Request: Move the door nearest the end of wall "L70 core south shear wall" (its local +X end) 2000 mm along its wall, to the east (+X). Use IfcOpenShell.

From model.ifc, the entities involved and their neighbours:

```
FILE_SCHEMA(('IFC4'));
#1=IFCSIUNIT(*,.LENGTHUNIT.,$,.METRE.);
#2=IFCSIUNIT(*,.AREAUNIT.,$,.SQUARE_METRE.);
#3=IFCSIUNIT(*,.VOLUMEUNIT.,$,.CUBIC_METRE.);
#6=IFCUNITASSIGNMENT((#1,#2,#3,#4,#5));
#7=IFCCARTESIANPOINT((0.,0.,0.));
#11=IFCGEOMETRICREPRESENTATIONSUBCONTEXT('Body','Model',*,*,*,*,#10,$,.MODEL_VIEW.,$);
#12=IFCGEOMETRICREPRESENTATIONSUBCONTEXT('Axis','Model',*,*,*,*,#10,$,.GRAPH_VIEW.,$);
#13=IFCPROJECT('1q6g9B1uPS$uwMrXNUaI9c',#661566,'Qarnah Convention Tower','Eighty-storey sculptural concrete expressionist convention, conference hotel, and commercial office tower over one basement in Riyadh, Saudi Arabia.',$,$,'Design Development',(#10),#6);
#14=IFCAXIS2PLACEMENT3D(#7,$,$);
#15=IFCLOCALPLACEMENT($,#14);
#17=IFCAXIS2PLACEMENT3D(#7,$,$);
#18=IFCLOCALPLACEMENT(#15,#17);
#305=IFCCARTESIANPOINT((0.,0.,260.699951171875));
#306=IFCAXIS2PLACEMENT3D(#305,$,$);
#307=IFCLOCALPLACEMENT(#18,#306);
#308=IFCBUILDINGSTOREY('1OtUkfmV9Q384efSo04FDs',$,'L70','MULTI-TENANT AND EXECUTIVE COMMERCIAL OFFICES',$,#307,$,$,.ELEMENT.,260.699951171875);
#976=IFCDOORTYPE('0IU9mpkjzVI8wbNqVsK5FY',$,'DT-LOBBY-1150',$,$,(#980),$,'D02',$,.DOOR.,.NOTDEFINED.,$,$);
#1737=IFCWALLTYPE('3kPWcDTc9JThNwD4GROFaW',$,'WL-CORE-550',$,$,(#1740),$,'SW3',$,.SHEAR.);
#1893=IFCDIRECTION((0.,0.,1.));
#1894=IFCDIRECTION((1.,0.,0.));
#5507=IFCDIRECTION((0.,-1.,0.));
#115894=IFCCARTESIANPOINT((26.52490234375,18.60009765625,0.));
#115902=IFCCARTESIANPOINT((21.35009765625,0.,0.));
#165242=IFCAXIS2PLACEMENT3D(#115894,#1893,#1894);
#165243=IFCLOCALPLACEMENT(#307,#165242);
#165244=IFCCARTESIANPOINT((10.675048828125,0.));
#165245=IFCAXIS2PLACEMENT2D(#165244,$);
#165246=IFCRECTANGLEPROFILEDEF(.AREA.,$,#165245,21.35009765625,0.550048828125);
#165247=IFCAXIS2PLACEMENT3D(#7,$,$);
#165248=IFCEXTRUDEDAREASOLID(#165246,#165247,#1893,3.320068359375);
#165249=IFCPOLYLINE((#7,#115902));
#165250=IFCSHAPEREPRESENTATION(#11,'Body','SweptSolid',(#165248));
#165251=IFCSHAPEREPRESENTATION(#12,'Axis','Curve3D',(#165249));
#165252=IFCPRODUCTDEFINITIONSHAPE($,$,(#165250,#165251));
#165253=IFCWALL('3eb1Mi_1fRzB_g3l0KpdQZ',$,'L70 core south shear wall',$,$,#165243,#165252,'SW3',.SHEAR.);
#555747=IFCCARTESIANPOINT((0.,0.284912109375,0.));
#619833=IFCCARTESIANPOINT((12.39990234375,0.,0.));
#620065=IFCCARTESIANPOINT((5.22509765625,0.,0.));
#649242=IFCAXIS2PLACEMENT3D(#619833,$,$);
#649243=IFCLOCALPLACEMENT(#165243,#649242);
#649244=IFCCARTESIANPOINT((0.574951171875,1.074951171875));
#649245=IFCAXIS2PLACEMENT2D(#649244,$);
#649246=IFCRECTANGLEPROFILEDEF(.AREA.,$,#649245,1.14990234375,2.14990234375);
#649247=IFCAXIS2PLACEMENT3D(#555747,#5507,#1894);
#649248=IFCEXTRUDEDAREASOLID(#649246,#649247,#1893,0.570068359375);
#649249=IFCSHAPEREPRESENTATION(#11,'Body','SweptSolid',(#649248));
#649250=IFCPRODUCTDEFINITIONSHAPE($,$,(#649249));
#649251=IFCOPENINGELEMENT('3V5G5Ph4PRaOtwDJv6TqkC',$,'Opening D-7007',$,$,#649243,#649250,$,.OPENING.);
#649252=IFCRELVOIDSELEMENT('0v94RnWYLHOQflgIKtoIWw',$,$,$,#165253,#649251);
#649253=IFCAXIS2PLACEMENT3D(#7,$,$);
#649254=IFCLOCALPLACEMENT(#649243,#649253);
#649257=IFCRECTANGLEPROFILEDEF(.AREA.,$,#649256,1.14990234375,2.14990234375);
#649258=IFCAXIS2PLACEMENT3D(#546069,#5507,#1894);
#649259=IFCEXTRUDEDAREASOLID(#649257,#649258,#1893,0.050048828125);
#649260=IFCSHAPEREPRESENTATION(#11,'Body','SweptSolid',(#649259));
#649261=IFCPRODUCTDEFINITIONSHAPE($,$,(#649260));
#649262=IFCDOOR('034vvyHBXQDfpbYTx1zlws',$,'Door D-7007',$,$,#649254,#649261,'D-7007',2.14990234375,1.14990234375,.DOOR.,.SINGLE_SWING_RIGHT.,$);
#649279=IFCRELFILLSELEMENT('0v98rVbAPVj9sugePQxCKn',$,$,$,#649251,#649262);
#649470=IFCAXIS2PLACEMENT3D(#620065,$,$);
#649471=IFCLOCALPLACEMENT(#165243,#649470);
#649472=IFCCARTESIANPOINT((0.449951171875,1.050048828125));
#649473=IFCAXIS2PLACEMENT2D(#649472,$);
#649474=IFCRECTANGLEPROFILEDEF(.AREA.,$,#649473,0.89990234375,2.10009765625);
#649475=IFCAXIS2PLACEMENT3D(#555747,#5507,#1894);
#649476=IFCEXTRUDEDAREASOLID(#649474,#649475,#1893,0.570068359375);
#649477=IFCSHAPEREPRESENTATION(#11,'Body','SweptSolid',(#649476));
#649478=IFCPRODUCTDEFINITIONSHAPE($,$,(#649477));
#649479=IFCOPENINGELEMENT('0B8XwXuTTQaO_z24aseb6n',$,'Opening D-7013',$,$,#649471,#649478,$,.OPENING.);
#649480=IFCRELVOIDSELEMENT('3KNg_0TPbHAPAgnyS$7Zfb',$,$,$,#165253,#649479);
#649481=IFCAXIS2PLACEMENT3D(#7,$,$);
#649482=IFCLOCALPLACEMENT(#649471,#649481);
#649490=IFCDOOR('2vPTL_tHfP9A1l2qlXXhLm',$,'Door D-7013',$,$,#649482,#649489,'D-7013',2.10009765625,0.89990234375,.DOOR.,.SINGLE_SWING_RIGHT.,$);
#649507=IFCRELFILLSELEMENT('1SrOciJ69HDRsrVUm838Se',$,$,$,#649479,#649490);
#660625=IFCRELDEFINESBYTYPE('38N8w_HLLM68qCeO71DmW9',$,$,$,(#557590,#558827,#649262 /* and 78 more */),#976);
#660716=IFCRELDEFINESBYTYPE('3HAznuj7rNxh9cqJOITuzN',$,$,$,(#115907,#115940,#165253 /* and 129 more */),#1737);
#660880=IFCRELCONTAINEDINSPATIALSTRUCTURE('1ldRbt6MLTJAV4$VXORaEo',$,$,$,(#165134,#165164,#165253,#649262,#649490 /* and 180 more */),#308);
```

```python
import ifcopenshell
import ifcopenshell.api.geometry
import ifcopenshell.util.placement

model = ifcopenshell.open("model.ifc")

door = model.by_guid("034vvyHBXQDfpbYTx1zlws")
opening = door.FillsVoids[0].RelatingOpeningElement
wall = opening.VoidsElements[0].RelatingBuildingElement

wall_matrix = ifcopenshell.util.placement.get_local_placement(wall.ObjectPlacement)
shift = wall_matrix[:3, 0] * 2.0
before = ifcopenshell.util.placement.get_local_placement(door.ObjectPlacement)[:3, 3].copy()

# The door is placed relative to its opening, so it follows when the opening moves.
matrix = ifcopenshell.util.placement.get_local_placement(opening.ObjectPlacement)
matrix[:3, 3] += shift
ifcopenshell.api.geometry.edit_object_placement(
    model, product=opening, matrix=matrix, is_si=False, should_transform_children=True
)

after = ifcopenshell.util.placement.get_local_placement(door.ObjectPlacement)[:3, 3]
print("door moved by", (after - before).round(3) + 0.0)

model.write("model_edited.ifc")
```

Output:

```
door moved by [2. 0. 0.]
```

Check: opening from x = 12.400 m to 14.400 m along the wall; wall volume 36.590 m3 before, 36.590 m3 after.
